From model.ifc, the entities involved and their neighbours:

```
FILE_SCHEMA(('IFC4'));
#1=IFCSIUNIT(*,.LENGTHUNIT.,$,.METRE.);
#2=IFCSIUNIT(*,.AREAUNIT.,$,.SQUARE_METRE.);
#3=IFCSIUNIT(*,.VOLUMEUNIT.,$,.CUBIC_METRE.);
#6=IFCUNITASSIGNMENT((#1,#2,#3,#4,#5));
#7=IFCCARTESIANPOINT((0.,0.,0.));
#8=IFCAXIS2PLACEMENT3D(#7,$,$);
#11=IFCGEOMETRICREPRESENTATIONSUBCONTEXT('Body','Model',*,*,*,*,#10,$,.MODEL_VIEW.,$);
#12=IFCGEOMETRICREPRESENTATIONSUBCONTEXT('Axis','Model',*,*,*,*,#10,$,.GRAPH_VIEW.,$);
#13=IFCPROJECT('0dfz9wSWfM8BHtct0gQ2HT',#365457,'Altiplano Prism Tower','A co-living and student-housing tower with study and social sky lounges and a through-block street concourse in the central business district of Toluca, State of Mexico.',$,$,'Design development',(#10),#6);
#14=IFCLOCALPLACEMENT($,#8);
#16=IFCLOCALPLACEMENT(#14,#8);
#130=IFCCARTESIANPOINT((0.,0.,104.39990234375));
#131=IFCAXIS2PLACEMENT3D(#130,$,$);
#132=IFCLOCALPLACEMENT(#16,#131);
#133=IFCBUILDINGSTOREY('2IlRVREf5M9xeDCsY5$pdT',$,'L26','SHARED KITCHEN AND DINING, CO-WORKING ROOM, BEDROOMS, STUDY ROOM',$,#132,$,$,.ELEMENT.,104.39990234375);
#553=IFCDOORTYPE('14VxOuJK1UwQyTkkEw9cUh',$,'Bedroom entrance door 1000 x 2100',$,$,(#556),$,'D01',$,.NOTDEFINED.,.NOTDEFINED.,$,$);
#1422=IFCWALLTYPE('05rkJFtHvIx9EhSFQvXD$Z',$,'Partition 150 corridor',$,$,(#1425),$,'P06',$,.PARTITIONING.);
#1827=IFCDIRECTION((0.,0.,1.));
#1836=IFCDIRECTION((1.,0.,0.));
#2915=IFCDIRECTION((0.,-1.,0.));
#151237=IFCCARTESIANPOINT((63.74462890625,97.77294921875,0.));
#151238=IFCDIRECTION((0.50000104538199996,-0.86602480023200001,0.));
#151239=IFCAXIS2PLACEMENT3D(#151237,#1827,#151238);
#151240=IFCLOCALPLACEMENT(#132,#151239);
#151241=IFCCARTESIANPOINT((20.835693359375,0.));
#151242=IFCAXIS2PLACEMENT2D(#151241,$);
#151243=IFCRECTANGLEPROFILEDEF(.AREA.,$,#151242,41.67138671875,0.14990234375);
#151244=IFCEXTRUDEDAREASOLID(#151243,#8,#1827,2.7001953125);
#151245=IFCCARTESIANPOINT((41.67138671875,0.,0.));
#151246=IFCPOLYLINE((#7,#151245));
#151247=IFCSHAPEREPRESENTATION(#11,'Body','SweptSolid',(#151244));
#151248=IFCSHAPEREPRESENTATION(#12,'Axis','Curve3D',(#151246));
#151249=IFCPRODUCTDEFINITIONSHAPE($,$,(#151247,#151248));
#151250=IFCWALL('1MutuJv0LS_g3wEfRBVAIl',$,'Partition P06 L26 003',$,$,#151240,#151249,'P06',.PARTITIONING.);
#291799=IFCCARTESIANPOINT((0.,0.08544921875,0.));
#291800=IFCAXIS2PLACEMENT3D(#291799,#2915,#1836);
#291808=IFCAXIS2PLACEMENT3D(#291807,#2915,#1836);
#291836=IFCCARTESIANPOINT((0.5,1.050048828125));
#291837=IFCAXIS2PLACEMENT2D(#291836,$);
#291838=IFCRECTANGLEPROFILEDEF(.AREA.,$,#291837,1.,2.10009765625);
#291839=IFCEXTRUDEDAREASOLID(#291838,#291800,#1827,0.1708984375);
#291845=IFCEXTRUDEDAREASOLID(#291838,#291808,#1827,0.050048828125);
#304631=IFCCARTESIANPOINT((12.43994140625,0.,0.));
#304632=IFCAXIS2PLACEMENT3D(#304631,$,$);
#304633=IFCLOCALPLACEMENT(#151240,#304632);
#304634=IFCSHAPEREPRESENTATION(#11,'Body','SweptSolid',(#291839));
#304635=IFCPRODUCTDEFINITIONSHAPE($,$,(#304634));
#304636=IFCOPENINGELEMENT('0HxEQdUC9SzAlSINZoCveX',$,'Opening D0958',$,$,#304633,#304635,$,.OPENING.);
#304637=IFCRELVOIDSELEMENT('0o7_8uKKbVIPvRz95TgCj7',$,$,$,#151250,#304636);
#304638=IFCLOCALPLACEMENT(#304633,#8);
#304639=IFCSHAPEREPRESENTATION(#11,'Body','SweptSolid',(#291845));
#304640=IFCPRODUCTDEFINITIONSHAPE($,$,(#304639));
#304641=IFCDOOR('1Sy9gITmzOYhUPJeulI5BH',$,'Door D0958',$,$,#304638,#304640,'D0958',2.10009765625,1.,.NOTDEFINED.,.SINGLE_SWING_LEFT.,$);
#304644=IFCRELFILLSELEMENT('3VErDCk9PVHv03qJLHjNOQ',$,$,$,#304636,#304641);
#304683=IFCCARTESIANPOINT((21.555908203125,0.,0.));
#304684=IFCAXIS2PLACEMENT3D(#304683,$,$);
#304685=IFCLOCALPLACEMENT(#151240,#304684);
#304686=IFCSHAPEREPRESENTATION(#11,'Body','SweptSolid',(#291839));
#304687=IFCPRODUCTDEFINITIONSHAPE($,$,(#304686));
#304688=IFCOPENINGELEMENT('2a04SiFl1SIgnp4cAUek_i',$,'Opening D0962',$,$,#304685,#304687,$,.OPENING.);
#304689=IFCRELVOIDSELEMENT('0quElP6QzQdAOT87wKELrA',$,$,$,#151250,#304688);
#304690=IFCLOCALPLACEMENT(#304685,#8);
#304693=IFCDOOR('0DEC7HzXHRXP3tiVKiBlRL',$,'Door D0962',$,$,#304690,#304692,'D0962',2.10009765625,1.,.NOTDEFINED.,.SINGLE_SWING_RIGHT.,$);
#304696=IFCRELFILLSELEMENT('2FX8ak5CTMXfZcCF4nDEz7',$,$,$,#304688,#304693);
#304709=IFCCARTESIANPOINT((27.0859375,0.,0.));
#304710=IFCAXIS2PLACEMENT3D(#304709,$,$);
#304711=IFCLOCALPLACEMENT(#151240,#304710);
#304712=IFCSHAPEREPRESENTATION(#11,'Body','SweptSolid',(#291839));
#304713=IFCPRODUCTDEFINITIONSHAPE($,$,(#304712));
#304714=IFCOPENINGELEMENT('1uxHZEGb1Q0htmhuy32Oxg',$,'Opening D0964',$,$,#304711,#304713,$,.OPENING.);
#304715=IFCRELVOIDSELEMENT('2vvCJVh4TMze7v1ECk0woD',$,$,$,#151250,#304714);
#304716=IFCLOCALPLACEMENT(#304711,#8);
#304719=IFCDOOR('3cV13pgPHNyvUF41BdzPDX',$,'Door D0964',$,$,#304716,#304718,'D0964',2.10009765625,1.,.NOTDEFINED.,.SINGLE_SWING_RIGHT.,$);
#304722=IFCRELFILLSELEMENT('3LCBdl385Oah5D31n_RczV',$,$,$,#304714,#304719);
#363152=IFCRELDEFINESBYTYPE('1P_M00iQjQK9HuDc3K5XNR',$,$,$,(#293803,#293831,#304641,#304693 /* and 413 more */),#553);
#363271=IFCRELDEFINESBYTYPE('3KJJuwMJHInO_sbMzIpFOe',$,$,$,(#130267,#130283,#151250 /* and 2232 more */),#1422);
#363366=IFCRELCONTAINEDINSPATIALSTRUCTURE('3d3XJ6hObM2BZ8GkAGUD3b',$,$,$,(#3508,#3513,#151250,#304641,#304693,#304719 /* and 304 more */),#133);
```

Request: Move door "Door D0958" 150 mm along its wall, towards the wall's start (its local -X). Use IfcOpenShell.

```python
import ifcopenshell
import ifcopenshell.api.geometry
import ifcopenshell.util.placement

model = ifcopenshell.open("model.ifc")

door = model.by_id(304641)
opening = door.FillsVoids[0].RelatingOpeningElement
wall = opening.VoidsElements[0].RelatingBuildingElement

wall_matrix = ifcopenshell.util.placement.get_local_placement(wall.ObjectPlacement)
shift = wall_matrix[:3, 0] * -0.15
before = ifcopenshell.util.placement.get_local_placement(door.ObjectPlacement)[:3, 3].copy()

# The door is placed relative to its opening, so it follows when the opening moves.
matrix = ifcopenshell.util.placement.get_local_placement(opening.ObjectPlacement)
matrix[:3, 3] += shift
ifcopenshell.api.geometry.edit_object_placement(
    model, product=opening, matrix=matrix, is_si=False, should_transform_children=True
)

after = ifcopenshell.util.placement.get_local_placement(door.ObjectPlacement)[:3, 3]
print("door moved by", (after - before).round(3) + 0.0)

model.write("model_updated.ifc")
```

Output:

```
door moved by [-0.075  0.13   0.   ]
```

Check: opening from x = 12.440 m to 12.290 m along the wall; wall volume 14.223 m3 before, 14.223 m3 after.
